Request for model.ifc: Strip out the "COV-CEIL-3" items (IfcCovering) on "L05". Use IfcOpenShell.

First a look at what the model holds.

```python
import ifcopenshell
import ifcopenshell.util.element

model = ifcopenshell.open("model.ifc")
print(model.schema)
storey = next(s for s in model.by_type("IfcBuildingStorey") if s.Name == "L05")
coverings = [e for e in ifcopenshell.util.element.get_decomposition(storey) if e.is_a("IfcCovering")]
seen = {}
for e in coverings:
    element_type = ifcopenshell.util.element.get_type(e)
    name = element_type.Name if element_type not in (None, e) else None
    seen[name] = seen.get(name, 0) + 1
for name, count in sorted(seen.items(), key=str):
    print(count, "x", name)
```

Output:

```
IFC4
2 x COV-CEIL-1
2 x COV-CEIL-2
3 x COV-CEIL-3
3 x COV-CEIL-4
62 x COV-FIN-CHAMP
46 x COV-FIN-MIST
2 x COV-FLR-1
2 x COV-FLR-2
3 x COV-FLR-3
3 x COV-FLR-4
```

```python
import ifcopenshell
import ifcopenshell.api.root
import ifcopenshell.util.element

model = ifcopenshell.open("model.ifc")

storey = next(s for s in model.by_type("IfcBuildingStorey") if s.Name == "L05")
coverings = [e for e in ifcopenshell.util.element.get_decomposition(storey) if e.is_a("IfcCovering")]
targets = [e for e in coverings if (t := ifcopenshell.util.element.get_type(e)) not in (None, e) and t.Name == "COV-CEIL-3"]

for e in targets:
    ifcopenshell.api.root.remove_product(model, product=e)
print(len(targets), "removed")

model.write("model_edited.ifc")
```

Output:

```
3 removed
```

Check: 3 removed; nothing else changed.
